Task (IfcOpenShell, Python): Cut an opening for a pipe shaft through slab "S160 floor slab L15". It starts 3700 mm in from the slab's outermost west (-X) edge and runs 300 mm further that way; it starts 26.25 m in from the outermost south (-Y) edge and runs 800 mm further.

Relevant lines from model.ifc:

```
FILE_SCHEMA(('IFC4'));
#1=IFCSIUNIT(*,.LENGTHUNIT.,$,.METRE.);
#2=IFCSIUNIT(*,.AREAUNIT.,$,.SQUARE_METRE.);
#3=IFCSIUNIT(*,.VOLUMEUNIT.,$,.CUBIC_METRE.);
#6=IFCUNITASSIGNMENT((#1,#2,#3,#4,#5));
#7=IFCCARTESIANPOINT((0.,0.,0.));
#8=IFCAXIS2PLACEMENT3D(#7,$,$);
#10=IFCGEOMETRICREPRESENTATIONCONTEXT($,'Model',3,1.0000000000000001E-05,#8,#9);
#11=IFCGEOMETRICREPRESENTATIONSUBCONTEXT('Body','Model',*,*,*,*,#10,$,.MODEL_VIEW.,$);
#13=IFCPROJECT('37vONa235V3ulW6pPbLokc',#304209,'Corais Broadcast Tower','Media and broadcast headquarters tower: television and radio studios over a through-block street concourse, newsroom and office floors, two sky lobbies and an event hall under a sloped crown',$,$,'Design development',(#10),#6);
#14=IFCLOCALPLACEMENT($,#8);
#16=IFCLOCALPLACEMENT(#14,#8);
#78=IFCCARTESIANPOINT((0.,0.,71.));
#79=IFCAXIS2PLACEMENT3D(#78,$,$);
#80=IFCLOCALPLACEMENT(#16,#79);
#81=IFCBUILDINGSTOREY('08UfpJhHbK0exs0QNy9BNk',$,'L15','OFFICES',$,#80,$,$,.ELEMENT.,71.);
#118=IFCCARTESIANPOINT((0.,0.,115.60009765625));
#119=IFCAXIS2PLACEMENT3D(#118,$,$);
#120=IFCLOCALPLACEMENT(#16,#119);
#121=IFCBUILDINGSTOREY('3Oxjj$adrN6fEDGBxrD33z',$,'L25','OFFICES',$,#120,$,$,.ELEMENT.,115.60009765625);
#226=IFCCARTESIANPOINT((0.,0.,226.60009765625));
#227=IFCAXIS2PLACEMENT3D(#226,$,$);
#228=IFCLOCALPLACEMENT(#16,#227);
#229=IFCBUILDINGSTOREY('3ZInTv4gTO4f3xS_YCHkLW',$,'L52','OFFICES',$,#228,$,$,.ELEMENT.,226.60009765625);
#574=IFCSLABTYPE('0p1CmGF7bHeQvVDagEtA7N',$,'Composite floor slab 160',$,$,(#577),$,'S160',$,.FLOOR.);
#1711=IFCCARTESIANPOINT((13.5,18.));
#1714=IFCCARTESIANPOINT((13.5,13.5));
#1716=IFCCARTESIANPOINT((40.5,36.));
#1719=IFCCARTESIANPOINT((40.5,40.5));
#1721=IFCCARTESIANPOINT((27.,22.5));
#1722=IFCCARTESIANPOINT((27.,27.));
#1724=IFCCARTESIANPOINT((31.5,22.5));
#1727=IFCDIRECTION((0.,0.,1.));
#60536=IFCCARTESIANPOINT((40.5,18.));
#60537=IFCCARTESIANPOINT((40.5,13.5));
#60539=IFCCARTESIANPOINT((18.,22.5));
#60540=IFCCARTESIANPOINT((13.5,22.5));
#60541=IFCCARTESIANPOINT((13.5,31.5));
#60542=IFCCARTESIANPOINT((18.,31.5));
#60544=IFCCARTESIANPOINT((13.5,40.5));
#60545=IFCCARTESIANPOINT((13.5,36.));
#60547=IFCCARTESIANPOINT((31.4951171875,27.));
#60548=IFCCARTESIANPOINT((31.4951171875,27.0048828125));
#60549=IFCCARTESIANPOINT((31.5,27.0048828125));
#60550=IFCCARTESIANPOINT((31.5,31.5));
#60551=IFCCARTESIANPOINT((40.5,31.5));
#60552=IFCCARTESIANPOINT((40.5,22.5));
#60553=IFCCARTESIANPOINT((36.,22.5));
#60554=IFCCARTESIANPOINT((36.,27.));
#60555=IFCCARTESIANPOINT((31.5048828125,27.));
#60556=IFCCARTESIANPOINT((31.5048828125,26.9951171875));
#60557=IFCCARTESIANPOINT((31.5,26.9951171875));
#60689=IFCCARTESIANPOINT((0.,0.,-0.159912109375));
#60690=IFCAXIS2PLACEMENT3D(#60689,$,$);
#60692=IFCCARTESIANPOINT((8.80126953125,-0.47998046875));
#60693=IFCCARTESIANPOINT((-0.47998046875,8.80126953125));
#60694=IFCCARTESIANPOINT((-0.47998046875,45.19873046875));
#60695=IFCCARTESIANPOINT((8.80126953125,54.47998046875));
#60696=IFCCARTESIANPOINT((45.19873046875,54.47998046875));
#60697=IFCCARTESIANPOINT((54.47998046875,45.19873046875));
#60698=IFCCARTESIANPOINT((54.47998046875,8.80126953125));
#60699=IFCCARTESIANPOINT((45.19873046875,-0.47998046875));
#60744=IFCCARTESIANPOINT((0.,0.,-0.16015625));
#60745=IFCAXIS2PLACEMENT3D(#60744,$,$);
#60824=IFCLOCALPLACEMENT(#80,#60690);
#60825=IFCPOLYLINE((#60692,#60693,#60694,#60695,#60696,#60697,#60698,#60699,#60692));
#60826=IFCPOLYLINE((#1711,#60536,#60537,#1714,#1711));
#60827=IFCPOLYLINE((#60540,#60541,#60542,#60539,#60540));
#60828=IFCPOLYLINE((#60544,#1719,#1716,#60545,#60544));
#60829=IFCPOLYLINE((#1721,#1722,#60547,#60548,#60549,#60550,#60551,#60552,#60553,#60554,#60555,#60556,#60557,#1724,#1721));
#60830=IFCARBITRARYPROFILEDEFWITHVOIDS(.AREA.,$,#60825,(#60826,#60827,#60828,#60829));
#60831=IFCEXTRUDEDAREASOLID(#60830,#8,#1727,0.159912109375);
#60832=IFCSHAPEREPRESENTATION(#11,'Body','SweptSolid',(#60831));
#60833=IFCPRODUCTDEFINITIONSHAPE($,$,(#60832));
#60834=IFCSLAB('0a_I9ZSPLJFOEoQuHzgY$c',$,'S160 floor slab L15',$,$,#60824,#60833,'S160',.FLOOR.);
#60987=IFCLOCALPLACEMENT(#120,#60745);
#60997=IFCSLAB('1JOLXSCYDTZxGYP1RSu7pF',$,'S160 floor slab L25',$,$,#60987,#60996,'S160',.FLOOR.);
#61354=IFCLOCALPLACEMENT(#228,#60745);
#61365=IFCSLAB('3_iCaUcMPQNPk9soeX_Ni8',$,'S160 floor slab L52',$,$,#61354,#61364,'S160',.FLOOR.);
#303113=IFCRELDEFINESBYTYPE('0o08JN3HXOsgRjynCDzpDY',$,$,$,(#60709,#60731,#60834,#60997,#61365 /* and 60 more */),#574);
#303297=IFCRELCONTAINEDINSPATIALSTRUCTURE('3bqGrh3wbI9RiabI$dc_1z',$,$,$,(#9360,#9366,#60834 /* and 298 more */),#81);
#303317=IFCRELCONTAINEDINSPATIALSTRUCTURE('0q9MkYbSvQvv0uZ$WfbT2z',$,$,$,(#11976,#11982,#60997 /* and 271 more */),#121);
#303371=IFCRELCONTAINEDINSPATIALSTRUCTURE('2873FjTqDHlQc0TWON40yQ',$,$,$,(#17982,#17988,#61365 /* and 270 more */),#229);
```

```python
import numpy as np
import ifcopenshell
import ifcopenshell.api.feature
import ifcopenshell.api.geometry
import ifcopenshell.api.root
import ifcopenshell.geom
import ifcopenshell.util.placement
import ifcopenshell.util.representation
import ifcopenshell.util.shape
import ifcopenshell.util.unit

model = ifcopenshell.open("model.ifc")
unit_scale = ifcopenshell.util.unit.calculate_unit_scale(model)
settings = ifcopenshell.geom.settings()


def volume(element):
    """Net volume in cubic metres, openings subtracted."""
    shape = ifcopenshell.geom.create_shape(settings, element)
    return ifcopenshell.util.shape.get_volume(shape.geometry)


slab = model.by_id(60834)
before = volume(slab)

# Extent in the slab's own axes, in metres. The edges named are its -X and -Y sides.
slab_shape = ifcopenshell.geom.create_shape(settings, slab)
vertices = ifcopenshell.util.shape.get_vertices(slab_shape.geometry)
x_min, y_min, bottom = vertices.min(axis=0)
top = vertices[:, 2].max()

opening = ifcopenshell.api.root.create_entity(model, ifc_class="IfcOpeningElement", name="Pipe shaft opening", predefined_type="OPENING")
context = ifcopenshell.util.representation.get_context(model, "Model", "Body", "MODEL_VIEW")
width, depth = 0.3, 0.8
outline = [(0.0, 0.0), (width, 0.0), (width, depth), (0.0, depth), (0.0, 0.0)]
# Overshoot both faces by 50 mm so the cut is clean.
shape = ifcopenshell.api.geometry.add_slab_representation(
    model, context=context, depth=top - bottom + 0.1, polyline=outline
)
ifcopenshell.api.geometry.assign_representation(model, product=opening, representation=shape)

matrix = ifcopenshell.util.placement.get_local_placement(slab.ObjectPlacement)
matrix[:, 3] = matrix @ np.append(np.array([x_min + 3.7, y_min + 26.25, bottom - 0.05]) / unit_scale, 1.0)
ifcopenshell.api.geometry.edit_object_placement(model, product=opening, matrix=matrix, is_si=False)
ifcopenshell.api.feature.add_feature(model, feature=opening, element=slab)

after = volume(slab)

print(f"slab volume {before:.3f} -> {after:.3f} m3")

model.write("model_rev.ifc")
```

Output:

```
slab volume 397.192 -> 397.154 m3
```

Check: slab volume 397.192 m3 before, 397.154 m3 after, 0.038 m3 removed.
